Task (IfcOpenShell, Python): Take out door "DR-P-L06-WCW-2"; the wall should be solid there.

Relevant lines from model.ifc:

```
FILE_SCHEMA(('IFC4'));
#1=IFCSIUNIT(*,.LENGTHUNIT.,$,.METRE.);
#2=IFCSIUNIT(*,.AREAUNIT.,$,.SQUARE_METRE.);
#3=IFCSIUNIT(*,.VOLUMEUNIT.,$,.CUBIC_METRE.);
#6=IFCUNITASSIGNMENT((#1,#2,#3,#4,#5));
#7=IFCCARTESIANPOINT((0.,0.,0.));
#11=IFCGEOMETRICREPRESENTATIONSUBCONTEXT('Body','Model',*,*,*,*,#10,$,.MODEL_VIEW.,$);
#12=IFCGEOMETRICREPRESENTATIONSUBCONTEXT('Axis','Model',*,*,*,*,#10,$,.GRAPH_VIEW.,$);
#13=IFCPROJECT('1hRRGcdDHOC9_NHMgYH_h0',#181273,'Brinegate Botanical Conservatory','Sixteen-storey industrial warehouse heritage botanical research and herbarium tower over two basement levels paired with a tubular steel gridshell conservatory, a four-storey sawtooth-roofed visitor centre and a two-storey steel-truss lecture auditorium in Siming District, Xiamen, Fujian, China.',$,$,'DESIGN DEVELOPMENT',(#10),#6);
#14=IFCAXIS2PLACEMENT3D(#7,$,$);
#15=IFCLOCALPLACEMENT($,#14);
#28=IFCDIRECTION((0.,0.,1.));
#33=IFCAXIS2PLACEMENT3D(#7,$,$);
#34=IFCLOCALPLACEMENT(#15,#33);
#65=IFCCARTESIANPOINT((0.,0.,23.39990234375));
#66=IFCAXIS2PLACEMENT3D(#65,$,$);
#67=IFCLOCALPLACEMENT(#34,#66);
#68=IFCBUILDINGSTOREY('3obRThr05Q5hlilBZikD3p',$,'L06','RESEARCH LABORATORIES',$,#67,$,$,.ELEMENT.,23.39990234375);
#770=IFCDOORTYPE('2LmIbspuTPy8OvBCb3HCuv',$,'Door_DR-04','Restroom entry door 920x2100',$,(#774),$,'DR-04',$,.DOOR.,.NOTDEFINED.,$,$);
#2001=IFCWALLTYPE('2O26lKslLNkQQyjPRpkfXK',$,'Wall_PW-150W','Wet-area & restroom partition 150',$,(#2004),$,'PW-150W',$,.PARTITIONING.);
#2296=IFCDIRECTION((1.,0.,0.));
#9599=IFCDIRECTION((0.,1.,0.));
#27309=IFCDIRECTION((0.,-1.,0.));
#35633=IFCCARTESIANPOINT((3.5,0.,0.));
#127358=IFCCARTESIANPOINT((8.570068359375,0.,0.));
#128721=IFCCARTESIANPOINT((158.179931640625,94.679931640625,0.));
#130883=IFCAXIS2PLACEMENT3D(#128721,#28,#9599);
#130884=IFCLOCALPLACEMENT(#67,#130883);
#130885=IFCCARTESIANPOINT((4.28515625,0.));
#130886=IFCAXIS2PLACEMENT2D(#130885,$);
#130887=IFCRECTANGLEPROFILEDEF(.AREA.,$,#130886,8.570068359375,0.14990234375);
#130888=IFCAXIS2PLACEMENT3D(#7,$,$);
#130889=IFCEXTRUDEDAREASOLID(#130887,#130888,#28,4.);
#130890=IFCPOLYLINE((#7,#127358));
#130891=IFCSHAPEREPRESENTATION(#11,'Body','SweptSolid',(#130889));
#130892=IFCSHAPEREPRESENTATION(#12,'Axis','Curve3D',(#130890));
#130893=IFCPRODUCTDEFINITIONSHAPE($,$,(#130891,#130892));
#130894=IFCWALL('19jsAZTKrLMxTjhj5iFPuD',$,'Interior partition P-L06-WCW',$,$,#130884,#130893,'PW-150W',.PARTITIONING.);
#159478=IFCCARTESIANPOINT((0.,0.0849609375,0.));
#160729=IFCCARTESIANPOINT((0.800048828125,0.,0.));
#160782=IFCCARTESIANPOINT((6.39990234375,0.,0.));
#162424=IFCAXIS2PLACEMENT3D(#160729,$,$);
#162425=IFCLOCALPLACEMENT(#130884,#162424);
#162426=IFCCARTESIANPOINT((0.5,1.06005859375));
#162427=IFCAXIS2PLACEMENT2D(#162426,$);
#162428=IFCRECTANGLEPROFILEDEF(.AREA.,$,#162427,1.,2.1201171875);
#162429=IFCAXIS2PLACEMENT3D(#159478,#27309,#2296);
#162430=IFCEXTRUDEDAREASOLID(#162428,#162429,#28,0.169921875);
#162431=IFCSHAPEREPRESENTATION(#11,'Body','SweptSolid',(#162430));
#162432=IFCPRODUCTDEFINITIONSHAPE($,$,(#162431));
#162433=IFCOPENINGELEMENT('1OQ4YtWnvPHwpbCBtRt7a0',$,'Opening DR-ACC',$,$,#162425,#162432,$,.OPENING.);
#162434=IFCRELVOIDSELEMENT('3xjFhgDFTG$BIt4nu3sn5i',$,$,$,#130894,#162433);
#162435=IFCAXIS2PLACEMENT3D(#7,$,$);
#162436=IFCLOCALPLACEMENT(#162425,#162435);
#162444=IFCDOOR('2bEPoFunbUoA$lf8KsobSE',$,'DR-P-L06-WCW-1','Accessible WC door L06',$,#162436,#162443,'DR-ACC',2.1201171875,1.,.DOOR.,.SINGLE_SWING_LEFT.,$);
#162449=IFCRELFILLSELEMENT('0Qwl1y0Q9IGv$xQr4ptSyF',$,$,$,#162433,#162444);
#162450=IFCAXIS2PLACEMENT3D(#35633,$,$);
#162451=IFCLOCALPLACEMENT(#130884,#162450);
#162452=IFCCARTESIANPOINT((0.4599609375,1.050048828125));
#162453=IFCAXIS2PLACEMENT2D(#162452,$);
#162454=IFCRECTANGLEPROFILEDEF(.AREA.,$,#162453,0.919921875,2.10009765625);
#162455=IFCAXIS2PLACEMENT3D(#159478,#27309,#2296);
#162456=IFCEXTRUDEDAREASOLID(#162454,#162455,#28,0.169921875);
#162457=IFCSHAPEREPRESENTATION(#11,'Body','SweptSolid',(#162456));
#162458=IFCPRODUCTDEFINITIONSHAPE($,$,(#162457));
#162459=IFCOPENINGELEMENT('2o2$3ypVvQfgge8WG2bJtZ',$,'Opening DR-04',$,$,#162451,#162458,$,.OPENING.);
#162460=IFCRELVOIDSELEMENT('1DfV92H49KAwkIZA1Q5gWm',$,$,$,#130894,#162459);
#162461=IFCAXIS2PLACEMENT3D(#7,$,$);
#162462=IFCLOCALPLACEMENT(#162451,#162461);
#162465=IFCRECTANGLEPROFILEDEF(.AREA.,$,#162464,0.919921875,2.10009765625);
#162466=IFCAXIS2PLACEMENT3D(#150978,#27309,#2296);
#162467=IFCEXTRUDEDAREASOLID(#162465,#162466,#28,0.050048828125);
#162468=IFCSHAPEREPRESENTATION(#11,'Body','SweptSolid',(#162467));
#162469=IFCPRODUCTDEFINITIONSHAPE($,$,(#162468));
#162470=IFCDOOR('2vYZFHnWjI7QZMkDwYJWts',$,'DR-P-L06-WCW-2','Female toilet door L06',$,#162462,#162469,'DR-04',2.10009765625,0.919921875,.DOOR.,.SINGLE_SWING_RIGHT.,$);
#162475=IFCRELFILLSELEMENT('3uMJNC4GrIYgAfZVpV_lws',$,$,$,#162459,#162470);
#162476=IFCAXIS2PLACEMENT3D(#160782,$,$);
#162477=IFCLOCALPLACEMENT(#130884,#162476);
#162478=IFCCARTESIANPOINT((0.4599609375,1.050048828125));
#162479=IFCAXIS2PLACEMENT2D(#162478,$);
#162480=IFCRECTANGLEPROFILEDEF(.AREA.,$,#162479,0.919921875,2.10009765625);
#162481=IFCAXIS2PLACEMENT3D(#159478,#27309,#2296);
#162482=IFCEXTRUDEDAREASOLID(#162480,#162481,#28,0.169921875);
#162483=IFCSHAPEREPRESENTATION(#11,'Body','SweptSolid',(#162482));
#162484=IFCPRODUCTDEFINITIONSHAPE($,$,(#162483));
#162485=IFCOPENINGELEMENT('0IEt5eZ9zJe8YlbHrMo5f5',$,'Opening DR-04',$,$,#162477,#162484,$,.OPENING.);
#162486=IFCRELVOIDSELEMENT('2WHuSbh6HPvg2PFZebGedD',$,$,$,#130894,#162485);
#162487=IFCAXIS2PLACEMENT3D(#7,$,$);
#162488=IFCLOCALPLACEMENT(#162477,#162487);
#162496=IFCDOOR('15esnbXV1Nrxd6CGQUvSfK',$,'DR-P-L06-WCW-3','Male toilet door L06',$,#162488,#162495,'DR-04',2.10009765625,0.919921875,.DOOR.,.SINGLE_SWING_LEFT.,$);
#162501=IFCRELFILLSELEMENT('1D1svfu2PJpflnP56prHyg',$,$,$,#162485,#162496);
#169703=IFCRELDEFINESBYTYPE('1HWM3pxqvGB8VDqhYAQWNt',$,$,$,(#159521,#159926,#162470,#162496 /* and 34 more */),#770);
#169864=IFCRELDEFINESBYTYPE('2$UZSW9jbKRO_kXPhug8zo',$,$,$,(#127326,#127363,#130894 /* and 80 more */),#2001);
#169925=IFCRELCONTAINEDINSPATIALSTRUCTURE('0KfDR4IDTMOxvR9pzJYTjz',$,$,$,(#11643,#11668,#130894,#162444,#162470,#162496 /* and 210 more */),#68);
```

```python
import ifcopenshell
import ifcopenshell.api.feature
import ifcopenshell.api.root
import ifcopenshell.geom
import ifcopenshell.util.shape

model = ifcopenshell.open("model.ifc")
settings = ifcopenshell.geom.settings()


def volume(element):
    """Net volume in cubic metres, openings subtracted."""
    shape = ifcopenshell.geom.create_shape(settings, element)
    return ifcopenshell.util.shape.get_volume(shape.geometry)


door = model.by_guid("2vYZFHnWjI7QZMkDwYJWts")
opening = door.FillsVoids[0].RelatingOpeningElement
wall = opening.VoidsElements[0].RelatingBuildingElement
before = volume(wall)

ifcopenshell.api.root.remove_product(model, product=door)
ifcopenshell.api.feature.remove_feature(model, feature=opening)

after = volume(wall)

print(f"wall volume {before:.3f} -> {after:.3f} m3")

model.write("model_rev.ifc")
```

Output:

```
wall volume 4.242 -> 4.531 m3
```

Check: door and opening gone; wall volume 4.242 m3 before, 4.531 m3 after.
